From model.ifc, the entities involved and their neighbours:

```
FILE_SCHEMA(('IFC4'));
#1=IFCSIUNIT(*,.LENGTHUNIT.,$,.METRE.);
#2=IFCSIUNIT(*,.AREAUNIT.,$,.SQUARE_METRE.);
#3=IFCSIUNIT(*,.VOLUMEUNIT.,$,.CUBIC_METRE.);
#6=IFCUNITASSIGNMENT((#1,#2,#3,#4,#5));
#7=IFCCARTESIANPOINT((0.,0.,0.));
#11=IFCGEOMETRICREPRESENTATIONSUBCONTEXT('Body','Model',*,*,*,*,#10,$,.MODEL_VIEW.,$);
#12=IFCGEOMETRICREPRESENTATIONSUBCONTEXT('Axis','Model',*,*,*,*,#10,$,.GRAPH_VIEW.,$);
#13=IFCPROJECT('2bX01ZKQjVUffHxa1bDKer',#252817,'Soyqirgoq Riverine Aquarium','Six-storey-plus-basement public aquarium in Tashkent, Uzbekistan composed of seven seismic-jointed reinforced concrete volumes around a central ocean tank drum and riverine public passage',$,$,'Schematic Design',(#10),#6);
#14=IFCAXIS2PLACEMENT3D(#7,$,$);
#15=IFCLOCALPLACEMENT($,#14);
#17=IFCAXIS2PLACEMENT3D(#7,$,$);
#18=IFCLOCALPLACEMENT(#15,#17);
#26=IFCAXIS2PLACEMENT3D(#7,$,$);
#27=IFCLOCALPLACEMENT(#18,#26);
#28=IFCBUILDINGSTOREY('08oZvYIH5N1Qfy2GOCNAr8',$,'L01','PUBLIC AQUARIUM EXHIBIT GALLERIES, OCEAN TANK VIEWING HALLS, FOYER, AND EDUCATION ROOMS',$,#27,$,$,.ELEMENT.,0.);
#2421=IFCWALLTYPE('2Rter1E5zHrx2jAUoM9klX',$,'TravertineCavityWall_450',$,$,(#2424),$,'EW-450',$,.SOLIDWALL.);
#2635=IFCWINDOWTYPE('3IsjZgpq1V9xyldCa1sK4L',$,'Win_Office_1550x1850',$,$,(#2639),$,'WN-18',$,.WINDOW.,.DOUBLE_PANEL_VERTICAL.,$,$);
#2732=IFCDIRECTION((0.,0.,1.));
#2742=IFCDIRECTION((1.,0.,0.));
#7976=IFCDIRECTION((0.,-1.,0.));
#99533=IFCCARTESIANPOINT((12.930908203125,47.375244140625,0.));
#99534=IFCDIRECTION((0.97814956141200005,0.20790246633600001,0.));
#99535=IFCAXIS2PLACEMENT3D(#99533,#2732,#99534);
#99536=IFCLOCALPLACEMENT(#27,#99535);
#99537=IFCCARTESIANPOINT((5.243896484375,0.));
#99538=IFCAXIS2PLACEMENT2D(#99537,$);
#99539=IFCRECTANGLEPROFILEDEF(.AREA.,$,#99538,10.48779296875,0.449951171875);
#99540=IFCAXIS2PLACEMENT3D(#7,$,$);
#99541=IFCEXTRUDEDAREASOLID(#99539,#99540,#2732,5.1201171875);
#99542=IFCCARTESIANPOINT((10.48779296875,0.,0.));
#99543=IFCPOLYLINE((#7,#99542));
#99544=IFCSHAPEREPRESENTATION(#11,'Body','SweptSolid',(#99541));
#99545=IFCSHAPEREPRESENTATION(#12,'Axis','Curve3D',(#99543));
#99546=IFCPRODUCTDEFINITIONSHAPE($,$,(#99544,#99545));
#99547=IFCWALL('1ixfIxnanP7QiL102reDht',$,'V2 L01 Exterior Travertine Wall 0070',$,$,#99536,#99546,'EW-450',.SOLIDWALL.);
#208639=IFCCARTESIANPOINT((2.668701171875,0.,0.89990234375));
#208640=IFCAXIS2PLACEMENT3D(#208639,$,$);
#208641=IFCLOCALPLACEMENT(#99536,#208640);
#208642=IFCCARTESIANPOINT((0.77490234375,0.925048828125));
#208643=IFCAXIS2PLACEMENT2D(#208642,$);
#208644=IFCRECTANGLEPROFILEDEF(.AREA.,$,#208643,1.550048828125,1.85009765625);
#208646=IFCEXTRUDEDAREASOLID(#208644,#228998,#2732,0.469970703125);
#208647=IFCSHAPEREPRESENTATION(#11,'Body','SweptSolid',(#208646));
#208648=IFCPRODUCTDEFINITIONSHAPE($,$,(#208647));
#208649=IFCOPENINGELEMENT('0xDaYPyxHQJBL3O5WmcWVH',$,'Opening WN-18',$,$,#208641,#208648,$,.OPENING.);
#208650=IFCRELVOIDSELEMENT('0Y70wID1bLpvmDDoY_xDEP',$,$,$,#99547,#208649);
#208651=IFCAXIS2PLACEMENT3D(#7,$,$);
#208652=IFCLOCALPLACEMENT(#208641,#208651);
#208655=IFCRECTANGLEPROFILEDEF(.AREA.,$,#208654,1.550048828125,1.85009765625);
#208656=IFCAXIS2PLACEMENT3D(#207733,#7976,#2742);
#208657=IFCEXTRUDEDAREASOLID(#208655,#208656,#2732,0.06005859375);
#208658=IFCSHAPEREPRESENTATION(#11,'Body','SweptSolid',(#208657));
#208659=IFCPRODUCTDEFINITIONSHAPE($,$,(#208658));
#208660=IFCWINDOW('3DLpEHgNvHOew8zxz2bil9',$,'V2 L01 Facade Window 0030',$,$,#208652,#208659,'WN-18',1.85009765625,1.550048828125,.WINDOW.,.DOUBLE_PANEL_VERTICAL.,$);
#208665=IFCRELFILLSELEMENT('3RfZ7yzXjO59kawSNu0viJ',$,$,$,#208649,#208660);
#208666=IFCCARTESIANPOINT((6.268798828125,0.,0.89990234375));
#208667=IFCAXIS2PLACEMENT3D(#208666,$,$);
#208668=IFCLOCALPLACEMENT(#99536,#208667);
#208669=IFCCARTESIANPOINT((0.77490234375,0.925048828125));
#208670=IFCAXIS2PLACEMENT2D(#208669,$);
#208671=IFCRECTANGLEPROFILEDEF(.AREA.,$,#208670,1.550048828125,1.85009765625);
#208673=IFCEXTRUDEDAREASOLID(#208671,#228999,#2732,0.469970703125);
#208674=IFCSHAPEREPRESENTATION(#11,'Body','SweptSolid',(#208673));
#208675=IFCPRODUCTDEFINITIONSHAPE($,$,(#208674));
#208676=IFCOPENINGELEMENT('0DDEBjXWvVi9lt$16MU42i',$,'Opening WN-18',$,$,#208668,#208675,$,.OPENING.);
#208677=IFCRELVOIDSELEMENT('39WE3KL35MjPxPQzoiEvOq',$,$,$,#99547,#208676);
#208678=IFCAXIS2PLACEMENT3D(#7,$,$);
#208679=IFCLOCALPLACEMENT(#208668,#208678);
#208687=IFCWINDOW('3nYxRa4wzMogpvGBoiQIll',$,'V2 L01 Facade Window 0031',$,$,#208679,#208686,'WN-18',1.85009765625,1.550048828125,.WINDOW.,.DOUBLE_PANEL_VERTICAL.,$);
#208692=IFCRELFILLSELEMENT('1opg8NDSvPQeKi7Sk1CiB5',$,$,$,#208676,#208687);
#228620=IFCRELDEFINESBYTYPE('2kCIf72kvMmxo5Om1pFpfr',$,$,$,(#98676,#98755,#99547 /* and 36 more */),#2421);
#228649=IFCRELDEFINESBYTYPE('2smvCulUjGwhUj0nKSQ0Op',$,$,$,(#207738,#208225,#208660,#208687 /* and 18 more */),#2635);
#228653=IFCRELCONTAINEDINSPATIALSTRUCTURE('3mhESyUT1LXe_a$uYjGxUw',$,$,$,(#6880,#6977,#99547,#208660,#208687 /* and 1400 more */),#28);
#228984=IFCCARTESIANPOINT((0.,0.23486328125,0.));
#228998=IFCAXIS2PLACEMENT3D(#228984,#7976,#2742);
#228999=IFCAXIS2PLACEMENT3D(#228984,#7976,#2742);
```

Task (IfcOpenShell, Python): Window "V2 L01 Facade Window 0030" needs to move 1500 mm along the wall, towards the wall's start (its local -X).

```python
import ifcopenshell
import ifcopenshell.api.geometry
import ifcopenshell.util.placement
import ifcopenshell.util.unit

model = ifcopenshell.open("model.ifc")
unit_scale = ifcopenshell.util.unit.calculate_unit_scale(model)

window = model.by_guid("3DLpEHgNvHOew8zxz2bil9")
opening = window.FillsVoids[0].RelatingOpeningElement
wall = opening.VoidsElements[0].RelatingBuildingElement

wall_matrix = ifcopenshell.util.placement.get_local_placement(wall.ObjectPlacement)
shift = wall_matrix[:3, 0] * -1.5 / unit_scale
before = ifcopenshell.util.placement.get_local_placement(window.ObjectPlacement)[:3, 3].copy()

# The window is placed relative to its opening, so it follows when the opening moves.
matrix = ifcopenshell.util.placement.get_local_placement(opening.ObjectPlacement)
matrix[:3, 3] += shift
ifcopenshell.api.geometry.edit_object_placement(
    model, product=opening, matrix=matrix, is_si=False, should_transform_children=True
)

after = ifcopenshell.util.placement.get_local_placement(window.ObjectPlacement)[:3, 3]
print("window moved by", (after - before).round(3) + 0.0)

model.write("model_edited.ifc")
```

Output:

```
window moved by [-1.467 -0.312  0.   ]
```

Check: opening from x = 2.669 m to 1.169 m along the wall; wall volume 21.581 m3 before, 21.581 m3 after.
